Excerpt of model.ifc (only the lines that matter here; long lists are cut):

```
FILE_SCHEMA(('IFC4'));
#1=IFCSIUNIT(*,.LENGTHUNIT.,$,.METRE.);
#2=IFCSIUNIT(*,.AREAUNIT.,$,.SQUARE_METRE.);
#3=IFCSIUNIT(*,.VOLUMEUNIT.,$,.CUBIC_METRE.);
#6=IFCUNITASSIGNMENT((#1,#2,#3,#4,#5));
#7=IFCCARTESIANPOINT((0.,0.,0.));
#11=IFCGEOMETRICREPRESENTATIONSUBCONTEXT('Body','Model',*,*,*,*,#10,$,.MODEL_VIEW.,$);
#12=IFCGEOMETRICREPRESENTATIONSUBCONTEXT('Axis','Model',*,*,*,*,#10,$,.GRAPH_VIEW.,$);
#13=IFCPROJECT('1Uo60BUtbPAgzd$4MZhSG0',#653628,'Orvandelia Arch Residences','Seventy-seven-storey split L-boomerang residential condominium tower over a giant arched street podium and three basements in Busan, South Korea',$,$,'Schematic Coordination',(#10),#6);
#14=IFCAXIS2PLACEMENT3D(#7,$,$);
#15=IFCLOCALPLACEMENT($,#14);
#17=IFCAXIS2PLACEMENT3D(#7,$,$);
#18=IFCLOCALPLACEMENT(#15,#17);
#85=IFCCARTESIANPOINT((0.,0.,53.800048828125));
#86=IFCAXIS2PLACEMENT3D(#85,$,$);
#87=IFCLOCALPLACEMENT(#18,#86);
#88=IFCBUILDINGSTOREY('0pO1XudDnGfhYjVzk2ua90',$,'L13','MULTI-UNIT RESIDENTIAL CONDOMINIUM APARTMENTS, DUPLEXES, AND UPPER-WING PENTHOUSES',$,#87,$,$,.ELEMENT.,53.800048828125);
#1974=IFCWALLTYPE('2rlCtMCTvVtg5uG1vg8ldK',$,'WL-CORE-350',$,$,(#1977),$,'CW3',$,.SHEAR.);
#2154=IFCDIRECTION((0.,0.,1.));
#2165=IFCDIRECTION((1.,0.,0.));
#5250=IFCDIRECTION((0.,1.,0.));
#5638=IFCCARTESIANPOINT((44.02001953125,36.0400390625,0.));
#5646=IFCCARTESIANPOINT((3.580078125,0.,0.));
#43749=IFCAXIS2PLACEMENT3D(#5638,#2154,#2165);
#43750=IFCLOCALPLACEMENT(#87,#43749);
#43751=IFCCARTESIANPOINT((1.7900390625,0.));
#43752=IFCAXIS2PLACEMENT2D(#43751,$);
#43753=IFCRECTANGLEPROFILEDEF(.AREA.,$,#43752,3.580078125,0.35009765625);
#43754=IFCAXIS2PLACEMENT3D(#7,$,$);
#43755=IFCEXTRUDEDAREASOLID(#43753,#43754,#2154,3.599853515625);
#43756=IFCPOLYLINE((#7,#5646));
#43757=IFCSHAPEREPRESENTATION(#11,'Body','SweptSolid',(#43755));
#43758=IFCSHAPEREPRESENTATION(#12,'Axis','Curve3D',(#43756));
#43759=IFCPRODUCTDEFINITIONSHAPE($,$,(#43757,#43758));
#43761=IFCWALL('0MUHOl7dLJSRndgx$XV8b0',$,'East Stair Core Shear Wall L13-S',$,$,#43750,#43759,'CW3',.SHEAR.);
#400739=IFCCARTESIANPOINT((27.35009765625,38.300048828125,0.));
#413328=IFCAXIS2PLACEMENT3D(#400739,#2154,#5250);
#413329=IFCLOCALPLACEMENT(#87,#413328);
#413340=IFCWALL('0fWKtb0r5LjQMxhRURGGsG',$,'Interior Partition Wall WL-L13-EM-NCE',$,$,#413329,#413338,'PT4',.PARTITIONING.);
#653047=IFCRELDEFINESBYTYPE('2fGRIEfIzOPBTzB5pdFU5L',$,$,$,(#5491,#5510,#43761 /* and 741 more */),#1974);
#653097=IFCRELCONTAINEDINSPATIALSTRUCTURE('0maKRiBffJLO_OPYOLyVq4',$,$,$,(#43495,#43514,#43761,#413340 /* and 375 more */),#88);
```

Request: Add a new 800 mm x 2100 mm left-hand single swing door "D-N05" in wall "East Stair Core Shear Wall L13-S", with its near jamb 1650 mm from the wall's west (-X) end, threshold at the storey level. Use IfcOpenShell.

```python
import numpy as np
import ifcopenshell
import ifcopenshell.api.feature
import ifcopenshell.api.geometry
import ifcopenshell.api.root
import ifcopenshell.api.spatial
import ifcopenshell.geom
import ifcopenshell.util.element
import ifcopenshell.util.placement
import ifcopenshell.util.representation
import ifcopenshell.util.shape
import ifcopenshell.util.unit

model = ifcopenshell.open("model.ifc")
unit_scale = ifcopenshell.util.unit.calculate_unit_scale(model)
settings = ifcopenshell.geom.settings()


def volume(element):
    """Net volume in cubic metres, openings subtracted."""
    shape = ifcopenshell.geom.create_shape(settings, element)
    return ifcopenshell.util.shape.get_volume(shape.geometry)


wall = model.by_id(43761)
storey = ifcopenshell.util.element.get_container(wall, ifc_class="IfcBuildingStorey")
context = ifcopenshell.util.representation.get_context(model, "Model", "Body", "MODEL_VIEW")
before = volume(wall)

width, height, from_end, sill = 0.8, 2.1, 1.65, 0.0  # metres

# The wall runs along its own X axis, and the end named is its -X end.
wall_shape = ifcopenshell.geom.create_shape(settings, wall)
x, y, z = ifcopenshell.util.shape.get_vertices(wall_shape.geometry).T
start = x.min() + from_end
face, thickness = float(y.min()), float(y.max() - y.min())
wall_matrix = ifcopenshell.util.placement.get_local_placement(wall.ObjectPlacement)
level = ifcopenshell.util.placement.get_local_placement(storey.ObjectPlacement)[2, 3]


def in_wall(x, y):
    """Placement at x, y metres in the wall's axes, at sill height."""
    matrix = wall_matrix.copy()
    matrix[:, 3] = wall_matrix @ np.array([x / unit_scale, y / unit_scale, 0.0, 1.0])
    matrix[2, 3] = level + sill / unit_scale
    return matrix


# Opening: a box that overshoots both wall faces by 50 mm.
opening = ifcopenshell.api.root.create_entity(model, ifc_class="IfcOpeningElement", predefined_type="OPENING")
box = ifcopenshell.api.geometry.add_wall_representation(
    model, context=context, length=width, height=height, thickness=thickness + 0.1
)
ifcopenshell.api.geometry.assign_representation(model, product=opening, representation=box)
ifcopenshell.api.geometry.edit_object_placement(model, product=opening, matrix=in_wall(start, face - 0.05), is_si=False)
ifcopenshell.api.feature.add_feature(model, feature=opening, element=wall)

door = ifcopenshell.api.root.create_entity(model, ifc_class="IfcDoor", name="D-N05", predefined_type="DOOR")
door.OverallWidth, door.OverallHeight = width / unit_scale, height / unit_scale
door.OperationType = "SINGLE_SWING_LEFT"
body = ifcopenshell.api.geometry.add_door_representation(
    model,
    context=context,
    overall_width=door.OverallWidth,
    overall_height=door.OverallHeight,
    operation_type="SINGLE_SWING_LEFT",
    lining_properties={"LiningDepth": thickness / unit_scale, "ThresholdDepth": thickness / unit_scale},
)
ifcopenshell.api.geometry.assign_representation(model, product=door, representation=body)
ifcopenshell.api.spatial.assign_container(model, products=[door], relating_structure=storey)
ifcopenshell.api.feature.add_filling(model, opening=opening, element=door)

# The lining spans the wall, so the door starts at the wall face.
ifcopenshell.api.geometry.edit_object_placement(model, product=door, matrix=in_wall(start, face), is_si=False)

after = volume(wall)

print(f"wall volume {before:.3f} -> {after:.3f} m3")

model.write("model_updated.ifc")
```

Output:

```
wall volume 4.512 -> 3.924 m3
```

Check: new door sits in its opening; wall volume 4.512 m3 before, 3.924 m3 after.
